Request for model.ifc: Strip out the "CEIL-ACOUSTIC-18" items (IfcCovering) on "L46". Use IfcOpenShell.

First a look at what the model holds.

```python
import ifcopenshell
import ifcopenshell.util.element

model = ifcopenshell.open("model.ifc")
print(model.schema)
storey = next(s for s in model.by_type("IfcBuildingStorey") if s.Name == "L46")
coverings = [e for e in ifcopenshell.util.element.get_decomposition(storey) if e.is_a("IfcCovering")]
seen = {}
for e in coverings:
    element_type = ifcopenshell.util.element.get_type(e)
    name = element_type.Name if element_type not in (None, e) else None
    seen[name] = seen.get(name, 0) + 1
for name, count in sorted(seen.items(), key=str):
    print(count, "x", name)
```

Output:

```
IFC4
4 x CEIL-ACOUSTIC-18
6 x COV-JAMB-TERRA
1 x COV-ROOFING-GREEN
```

```python
import ifcopenshell
import ifcopenshell.api.root
import ifcopenshell.util.element

model = ifcopenshell.open("model.ifc")

storey = next(s for s in model.by_type("IfcBuildingStorey") if s.Name == "L46")
coverings = [e for e in ifcopenshell.util.element.get_decomposition(storey) if e.is_a("IfcCovering")]
targets = [e for e in coverings if (t := ifcopenshell.util.element.get_type(e)) not in (None, e) and t.Name == "CEIL-ACOUSTIC-18"]

for e in targets:
    ifcopenshell.api.root.remove_product(model, product=e)
print(len(targets), "removed")

model.write("model_edited.ifc")
```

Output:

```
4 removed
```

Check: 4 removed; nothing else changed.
